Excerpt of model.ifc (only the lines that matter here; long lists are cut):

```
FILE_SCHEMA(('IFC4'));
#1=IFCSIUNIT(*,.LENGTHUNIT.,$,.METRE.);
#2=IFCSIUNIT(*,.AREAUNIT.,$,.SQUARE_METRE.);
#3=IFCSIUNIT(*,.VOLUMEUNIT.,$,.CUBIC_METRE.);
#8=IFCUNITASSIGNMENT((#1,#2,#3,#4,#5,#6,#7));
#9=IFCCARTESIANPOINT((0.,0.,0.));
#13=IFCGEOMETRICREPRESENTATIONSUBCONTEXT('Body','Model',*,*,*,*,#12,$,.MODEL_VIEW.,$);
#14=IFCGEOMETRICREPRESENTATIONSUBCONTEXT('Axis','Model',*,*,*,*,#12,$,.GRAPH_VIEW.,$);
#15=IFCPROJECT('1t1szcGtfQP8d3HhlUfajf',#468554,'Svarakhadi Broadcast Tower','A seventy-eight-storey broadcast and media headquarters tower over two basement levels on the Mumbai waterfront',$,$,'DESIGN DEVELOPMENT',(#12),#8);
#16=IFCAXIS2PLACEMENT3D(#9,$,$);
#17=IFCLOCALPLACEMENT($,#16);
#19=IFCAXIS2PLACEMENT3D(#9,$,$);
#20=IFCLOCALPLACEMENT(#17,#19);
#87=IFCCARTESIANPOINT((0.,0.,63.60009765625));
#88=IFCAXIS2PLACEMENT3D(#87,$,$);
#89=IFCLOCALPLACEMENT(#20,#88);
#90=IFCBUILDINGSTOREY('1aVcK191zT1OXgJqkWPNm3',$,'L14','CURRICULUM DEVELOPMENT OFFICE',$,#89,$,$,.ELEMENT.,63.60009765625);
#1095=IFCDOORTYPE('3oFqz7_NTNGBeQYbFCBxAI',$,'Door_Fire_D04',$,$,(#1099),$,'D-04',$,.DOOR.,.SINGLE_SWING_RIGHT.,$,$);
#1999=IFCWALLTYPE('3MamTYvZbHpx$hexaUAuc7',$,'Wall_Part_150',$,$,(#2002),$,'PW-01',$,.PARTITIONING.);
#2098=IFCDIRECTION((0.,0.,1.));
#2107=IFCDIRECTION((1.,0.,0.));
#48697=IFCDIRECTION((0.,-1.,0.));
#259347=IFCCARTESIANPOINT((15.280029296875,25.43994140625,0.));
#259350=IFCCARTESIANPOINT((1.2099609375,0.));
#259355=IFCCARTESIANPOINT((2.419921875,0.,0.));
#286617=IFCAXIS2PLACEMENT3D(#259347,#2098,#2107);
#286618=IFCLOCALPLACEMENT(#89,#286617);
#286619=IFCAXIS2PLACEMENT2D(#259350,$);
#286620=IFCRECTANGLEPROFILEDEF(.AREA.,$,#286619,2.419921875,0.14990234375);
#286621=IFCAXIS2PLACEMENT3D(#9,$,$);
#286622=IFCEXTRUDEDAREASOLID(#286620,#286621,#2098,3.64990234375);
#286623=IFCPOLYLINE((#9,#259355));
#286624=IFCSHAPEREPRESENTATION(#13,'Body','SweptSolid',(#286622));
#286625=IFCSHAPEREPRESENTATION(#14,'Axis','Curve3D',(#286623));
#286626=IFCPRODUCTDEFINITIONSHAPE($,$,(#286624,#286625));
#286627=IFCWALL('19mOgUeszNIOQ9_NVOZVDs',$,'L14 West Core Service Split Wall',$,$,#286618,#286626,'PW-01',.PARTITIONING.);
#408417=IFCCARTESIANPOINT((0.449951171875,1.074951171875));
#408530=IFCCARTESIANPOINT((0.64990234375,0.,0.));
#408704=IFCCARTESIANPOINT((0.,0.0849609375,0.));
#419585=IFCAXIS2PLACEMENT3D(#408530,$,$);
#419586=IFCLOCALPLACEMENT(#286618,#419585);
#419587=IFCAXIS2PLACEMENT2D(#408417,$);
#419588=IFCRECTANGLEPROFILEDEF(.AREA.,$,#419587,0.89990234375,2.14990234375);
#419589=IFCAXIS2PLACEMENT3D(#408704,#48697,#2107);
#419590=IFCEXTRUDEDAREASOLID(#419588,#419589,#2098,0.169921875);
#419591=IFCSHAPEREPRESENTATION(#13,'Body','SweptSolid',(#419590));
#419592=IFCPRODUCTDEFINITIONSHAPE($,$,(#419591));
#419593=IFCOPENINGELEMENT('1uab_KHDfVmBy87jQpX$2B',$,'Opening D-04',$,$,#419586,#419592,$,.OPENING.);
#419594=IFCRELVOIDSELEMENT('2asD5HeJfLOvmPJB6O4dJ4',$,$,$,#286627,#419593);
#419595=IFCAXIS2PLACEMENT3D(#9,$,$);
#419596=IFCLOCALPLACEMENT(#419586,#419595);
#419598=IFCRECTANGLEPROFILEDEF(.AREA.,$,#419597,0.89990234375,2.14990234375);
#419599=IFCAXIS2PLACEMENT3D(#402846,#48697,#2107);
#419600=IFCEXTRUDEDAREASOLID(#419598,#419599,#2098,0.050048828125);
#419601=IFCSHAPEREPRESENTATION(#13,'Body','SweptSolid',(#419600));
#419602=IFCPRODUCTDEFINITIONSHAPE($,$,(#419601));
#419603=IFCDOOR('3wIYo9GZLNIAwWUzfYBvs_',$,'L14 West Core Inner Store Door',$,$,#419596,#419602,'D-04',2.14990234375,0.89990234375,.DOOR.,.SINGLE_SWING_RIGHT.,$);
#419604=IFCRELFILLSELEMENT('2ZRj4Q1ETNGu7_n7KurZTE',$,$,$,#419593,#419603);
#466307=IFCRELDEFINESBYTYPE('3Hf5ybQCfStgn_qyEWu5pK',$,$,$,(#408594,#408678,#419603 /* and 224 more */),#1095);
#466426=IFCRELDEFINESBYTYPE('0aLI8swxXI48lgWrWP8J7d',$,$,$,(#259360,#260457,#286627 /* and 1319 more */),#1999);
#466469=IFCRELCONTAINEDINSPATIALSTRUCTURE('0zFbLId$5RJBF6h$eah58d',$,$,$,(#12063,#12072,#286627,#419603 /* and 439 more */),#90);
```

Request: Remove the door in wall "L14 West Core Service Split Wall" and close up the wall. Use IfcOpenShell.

```python
import ifcopenshell
import ifcopenshell.api.feature
import ifcopenshell.api.root
import ifcopenshell.geom
import ifcopenshell.util.shape

model = ifcopenshell.open("model.ifc")
settings = ifcopenshell.geom.settings()


def volume(element):
    """Net volume in cubic metres, openings subtracted."""
    shape = ifcopenshell.geom.create_shape(settings, element)
    return ifcopenshell.util.shape.get_volume(shape.geometry)


door = model.by_guid("3wIYo9GZLNIAwWUzfYBvs_")
opening = door.FillsVoids[0].RelatingOpeningElement
wall = opening.VoidsElements[0].RelatingBuildingElement
before = volume(wall)

ifcopenshell.api.root.remove_product(model, product=door)
ifcopenshell.api.feature.remove_feature(model, feature=opening)

after = volume(wall)

print(f"wall volume {before:.3f} -> {after:.3f} m3")

model.write("model_rev.ifc")
```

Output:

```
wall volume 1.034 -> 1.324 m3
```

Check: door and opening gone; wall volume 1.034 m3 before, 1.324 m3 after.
